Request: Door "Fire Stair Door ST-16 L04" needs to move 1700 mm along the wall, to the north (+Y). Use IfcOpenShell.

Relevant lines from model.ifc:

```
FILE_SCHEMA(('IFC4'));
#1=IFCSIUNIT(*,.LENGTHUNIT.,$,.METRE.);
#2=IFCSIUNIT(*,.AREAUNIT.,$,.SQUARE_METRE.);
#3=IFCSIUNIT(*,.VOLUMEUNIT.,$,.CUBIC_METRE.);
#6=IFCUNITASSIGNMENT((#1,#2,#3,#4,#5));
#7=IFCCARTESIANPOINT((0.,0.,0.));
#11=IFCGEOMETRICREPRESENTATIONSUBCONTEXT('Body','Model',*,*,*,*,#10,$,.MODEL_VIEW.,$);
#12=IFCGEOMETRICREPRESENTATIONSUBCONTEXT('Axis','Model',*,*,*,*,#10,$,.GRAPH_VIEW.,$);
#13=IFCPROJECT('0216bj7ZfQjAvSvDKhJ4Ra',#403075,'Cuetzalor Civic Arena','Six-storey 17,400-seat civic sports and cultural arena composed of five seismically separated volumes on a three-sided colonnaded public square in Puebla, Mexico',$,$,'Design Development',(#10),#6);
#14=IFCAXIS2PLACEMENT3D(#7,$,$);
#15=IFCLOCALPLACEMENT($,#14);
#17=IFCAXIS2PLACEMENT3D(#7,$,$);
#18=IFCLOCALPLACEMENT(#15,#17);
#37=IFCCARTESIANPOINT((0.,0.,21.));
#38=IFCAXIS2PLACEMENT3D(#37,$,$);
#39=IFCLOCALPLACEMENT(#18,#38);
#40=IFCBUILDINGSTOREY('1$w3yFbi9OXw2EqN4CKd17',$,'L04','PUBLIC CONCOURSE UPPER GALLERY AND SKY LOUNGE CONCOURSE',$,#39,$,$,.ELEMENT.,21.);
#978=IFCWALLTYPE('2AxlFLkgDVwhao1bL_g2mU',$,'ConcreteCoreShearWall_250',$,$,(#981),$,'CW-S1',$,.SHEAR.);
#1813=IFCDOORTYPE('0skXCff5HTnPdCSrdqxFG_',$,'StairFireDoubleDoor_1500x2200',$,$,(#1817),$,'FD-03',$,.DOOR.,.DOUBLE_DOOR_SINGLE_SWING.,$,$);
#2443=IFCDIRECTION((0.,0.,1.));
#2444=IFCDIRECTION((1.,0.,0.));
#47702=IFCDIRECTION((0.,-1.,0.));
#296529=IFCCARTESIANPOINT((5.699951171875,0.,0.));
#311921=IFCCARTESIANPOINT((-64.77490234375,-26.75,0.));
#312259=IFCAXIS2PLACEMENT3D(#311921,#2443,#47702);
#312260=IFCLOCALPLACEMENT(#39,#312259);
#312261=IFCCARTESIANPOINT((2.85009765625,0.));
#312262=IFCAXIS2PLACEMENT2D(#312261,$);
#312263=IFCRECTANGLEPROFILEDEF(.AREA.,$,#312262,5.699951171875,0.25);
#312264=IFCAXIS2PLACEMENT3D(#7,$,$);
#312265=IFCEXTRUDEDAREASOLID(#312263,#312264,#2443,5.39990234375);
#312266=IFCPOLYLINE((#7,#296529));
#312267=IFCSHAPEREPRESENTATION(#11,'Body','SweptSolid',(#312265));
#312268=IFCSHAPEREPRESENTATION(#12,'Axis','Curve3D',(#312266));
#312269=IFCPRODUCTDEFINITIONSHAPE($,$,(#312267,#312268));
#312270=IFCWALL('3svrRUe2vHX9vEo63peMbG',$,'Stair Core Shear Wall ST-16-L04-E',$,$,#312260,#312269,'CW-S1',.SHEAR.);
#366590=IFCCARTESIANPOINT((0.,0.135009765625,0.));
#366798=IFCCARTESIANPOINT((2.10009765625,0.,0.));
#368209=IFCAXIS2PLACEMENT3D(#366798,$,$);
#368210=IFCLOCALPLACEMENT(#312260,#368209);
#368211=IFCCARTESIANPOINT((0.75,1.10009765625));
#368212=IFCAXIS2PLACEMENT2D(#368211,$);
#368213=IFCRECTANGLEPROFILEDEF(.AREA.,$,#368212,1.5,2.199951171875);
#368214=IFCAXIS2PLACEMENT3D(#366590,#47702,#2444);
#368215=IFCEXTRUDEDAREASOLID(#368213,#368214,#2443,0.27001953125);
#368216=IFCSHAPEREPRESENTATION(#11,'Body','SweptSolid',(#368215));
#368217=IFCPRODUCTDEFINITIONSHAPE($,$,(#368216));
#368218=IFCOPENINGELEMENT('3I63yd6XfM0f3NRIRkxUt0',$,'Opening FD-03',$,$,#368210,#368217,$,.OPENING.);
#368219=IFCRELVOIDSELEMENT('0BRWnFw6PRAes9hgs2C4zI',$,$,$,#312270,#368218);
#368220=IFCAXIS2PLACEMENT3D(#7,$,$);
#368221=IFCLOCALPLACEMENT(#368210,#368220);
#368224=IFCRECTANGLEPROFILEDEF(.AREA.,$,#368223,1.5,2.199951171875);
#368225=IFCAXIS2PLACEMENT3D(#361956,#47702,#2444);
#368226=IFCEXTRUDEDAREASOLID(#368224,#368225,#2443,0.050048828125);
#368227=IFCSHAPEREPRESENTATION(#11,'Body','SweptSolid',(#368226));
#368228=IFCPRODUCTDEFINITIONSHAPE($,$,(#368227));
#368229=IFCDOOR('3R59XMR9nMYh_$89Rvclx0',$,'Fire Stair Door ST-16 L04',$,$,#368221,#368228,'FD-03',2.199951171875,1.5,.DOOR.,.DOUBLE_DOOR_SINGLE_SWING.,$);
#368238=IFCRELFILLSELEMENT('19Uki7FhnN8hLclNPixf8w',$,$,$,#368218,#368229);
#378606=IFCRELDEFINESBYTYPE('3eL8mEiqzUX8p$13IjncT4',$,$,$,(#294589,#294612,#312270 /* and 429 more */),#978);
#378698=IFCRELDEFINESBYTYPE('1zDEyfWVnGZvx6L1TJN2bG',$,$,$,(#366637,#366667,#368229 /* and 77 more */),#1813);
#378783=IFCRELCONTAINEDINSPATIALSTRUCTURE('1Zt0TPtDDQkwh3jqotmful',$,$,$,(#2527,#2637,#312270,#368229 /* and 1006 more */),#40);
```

```python
import ifcopenshell
import ifcopenshell.api.geometry
import ifcopenshell.util.placement
import ifcopenshell.util.unit

model = ifcopenshell.open("model.ifc")
unit_scale = ifcopenshell.util.unit.calculate_unit_scale(model)

door = model.by_guid("3R59XMR9nMYh_$89Rvclx0")
opening = door.FillsVoids[0].RelatingOpeningElement
wall = opening.VoidsElements[0].RelatingBuildingElement

wall_matrix = ifcopenshell.util.placement.get_local_placement(wall.ObjectPlacement)
shift = wall_matrix[:3, 0] * -1.7 / unit_scale
before = ifcopenshell.util.placement.get_local_placement(door.ObjectPlacement)[:3, 3].copy()

# The door is placed relative to its opening, so it follows when the opening moves.
matrix = ifcopenshell.util.placement.get_local_placement(opening.ObjectPlacement)
matrix[:3, 3] += shift
ifcopenshell.api.geometry.edit_object_placement(
    model, product=opening, matrix=matrix, is_si=False, should_transform_children=True
)

after = ifcopenshell.util.placement.get_local_placement(door.ObjectPlacement)[:3, 3]
print("door moved by", (after - before).round(3) + 0.0)

model.write("model_edited.ifc")
```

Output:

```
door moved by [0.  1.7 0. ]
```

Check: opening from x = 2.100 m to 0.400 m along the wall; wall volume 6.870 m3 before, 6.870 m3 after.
